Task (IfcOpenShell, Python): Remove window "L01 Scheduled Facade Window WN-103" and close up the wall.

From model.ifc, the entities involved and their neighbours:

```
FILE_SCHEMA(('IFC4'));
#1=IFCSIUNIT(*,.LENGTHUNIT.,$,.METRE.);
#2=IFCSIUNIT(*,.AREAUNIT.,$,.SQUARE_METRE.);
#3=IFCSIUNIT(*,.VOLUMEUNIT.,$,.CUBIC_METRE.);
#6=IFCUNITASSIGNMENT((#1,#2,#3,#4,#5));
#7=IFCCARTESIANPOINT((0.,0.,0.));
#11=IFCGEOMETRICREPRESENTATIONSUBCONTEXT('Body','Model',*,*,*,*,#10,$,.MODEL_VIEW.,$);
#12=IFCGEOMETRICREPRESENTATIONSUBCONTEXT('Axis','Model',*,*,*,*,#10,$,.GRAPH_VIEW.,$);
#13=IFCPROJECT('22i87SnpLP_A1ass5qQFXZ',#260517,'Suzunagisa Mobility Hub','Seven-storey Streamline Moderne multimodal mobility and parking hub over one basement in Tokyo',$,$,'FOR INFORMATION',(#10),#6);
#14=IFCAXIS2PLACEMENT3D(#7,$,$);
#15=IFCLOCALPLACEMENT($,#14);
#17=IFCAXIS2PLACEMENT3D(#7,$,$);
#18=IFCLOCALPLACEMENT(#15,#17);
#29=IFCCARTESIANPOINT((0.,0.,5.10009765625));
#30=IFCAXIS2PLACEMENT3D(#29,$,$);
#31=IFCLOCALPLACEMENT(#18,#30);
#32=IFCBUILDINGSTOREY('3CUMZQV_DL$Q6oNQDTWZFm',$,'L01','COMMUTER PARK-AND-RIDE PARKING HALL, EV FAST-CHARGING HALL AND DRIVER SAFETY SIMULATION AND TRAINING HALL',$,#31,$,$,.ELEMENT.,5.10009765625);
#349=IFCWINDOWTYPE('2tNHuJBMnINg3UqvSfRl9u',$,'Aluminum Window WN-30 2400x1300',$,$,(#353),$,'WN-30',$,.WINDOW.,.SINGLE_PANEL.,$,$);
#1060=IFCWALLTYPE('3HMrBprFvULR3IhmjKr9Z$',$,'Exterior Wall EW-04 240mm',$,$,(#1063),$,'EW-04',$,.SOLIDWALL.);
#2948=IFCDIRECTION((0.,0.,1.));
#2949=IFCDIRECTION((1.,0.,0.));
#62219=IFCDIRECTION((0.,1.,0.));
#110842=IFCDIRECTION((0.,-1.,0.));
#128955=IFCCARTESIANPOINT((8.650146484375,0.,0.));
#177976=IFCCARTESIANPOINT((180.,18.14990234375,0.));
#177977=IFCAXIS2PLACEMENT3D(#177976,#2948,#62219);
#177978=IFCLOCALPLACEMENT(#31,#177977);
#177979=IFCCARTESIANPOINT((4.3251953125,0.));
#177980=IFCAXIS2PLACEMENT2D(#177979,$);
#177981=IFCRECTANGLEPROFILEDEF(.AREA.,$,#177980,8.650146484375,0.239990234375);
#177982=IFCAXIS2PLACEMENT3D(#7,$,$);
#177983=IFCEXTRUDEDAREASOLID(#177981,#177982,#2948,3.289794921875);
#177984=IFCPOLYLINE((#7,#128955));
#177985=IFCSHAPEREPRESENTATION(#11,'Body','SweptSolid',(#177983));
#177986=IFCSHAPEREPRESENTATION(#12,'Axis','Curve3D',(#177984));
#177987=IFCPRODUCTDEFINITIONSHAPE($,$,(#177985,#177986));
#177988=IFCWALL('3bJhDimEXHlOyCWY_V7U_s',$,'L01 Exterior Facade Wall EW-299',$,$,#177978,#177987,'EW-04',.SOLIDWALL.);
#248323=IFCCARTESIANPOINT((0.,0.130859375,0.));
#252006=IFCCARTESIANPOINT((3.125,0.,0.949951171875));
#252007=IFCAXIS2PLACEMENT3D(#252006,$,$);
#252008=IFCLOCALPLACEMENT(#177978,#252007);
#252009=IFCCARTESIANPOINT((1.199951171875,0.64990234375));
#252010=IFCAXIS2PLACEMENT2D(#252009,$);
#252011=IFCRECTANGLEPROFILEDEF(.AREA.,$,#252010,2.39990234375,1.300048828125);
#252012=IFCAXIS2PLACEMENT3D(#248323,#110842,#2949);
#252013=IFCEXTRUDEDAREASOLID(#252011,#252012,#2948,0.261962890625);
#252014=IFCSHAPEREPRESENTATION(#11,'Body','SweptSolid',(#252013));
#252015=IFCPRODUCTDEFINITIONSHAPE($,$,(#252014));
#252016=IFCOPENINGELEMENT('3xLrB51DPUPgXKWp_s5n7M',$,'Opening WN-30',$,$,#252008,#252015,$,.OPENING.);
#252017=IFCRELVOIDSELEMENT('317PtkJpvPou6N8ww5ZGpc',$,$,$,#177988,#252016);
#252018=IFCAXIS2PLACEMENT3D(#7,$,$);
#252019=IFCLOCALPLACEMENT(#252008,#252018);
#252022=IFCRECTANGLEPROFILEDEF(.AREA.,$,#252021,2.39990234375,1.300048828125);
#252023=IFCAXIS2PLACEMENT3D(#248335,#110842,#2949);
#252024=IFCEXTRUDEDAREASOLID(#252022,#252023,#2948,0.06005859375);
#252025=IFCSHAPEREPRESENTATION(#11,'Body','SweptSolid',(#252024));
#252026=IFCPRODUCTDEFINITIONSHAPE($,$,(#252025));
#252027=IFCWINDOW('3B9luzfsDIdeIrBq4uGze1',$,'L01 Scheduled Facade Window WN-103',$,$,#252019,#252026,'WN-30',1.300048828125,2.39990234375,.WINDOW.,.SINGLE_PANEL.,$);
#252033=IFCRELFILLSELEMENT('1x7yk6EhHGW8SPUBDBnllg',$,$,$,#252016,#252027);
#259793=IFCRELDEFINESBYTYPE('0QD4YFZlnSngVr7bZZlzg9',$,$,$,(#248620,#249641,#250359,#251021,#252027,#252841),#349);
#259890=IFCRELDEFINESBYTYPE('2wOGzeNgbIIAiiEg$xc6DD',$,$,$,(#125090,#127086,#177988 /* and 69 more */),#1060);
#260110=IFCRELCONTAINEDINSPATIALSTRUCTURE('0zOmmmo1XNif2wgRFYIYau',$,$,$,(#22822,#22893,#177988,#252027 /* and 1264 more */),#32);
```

```python
import ifcopenshell
import ifcopenshell.api.feature
import ifcopenshell.api.root
import ifcopenshell.geom
import ifcopenshell.util.shape

model = ifcopenshell.open("model.ifc")
settings = ifcopenshell.geom.settings()


def volume(element):
    """Net volume in cubic metres, openings subtracted."""
    shape = ifcopenshell.geom.create_shape(settings, element)
    return ifcopenshell.util.shape.get_volume(shape.geometry)


window = model.by_guid("3B9luzfsDIdeIrBq4uGze1")
opening = window.FillsVoids[0].RelatingOpeningElement
wall = opening.VoidsElements[0].RelatingBuildingElement
before = volume(wall)

ifcopenshell.api.root.remove_product(model, product=window)
ifcopenshell.api.feature.remove_feature(model, feature=opening)

after = volume(wall)

print(f"wall volume {before:.3f} -> {after:.3f} m3")

model.write("model_updated.ifc")
```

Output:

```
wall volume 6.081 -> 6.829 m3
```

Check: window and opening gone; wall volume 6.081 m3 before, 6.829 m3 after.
